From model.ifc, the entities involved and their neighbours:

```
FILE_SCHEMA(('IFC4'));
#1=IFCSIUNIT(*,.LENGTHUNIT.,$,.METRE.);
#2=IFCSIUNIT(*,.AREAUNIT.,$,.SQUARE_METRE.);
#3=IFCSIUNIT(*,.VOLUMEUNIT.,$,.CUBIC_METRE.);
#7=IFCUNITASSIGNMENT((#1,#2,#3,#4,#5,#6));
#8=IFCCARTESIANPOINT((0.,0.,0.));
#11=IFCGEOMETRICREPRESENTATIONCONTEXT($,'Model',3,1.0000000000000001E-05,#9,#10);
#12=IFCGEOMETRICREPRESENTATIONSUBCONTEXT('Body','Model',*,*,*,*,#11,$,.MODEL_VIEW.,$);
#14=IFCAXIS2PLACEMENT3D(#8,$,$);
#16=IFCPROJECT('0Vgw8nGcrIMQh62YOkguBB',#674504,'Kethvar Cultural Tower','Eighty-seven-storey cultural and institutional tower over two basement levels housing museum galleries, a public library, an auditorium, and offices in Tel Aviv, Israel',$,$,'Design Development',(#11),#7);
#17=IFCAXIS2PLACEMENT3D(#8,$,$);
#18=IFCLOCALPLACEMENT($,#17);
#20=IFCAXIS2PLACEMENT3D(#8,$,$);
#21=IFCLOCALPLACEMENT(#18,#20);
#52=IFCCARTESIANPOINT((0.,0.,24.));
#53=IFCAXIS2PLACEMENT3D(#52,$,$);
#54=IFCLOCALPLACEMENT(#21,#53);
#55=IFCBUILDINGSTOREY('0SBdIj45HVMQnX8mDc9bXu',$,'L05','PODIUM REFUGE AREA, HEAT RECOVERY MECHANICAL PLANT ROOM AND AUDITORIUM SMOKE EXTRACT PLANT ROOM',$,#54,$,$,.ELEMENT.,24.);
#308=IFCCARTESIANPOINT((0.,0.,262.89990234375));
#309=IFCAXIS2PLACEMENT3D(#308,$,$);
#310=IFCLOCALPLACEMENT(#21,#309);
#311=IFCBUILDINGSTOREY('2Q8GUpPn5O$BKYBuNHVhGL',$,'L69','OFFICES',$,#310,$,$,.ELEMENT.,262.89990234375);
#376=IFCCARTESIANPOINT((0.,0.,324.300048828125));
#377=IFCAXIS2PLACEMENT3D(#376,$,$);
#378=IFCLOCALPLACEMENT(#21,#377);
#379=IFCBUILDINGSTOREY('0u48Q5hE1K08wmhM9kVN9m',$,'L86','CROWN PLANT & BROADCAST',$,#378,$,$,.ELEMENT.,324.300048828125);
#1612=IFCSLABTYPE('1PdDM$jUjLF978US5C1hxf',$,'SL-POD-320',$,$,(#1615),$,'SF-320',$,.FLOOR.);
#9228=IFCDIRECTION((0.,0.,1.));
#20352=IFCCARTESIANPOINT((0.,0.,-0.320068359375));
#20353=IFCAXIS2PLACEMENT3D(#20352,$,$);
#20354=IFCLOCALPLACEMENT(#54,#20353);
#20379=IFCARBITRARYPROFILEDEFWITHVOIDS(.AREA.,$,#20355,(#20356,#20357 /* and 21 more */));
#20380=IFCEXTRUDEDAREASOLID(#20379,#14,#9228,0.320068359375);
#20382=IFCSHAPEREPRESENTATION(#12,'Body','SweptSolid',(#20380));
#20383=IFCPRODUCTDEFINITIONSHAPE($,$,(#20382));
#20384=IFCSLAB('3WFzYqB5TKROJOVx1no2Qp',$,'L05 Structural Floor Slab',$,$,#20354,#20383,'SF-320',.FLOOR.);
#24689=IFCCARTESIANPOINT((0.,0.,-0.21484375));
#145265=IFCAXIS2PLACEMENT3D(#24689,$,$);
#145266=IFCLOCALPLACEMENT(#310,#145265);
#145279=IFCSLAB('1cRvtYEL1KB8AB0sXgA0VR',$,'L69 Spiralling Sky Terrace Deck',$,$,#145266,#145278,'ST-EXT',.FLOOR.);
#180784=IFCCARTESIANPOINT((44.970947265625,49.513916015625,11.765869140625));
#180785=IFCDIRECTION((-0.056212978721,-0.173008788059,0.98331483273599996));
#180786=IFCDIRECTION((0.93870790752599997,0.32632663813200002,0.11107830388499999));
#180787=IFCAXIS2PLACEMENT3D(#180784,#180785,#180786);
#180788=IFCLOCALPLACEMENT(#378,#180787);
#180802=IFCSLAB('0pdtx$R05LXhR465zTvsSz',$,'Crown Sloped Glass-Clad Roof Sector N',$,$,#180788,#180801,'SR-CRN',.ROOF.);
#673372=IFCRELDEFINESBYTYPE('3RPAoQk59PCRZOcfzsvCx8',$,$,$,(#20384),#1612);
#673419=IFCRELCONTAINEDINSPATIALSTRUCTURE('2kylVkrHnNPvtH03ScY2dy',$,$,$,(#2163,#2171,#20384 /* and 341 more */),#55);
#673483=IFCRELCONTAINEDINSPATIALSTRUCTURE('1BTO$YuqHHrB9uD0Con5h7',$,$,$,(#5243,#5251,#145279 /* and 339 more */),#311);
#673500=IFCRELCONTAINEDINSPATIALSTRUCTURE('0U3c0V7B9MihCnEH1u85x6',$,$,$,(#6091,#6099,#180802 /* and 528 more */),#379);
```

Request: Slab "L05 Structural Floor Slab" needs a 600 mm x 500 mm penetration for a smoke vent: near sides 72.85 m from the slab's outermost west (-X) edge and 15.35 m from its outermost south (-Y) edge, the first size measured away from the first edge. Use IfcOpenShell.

```python
import numpy as np
import ifcopenshell
import ifcopenshell.api.feature
import ifcopenshell.api.geometry
import ifcopenshell.api.root
import ifcopenshell.geom
import ifcopenshell.util.placement
import ifcopenshell.util.representation
import ifcopenshell.util.shape
import ifcopenshell.util.unit

model = ifcopenshell.open("model.ifc")
unit_scale = ifcopenshell.util.unit.calculate_unit_scale(model)
settings = ifcopenshell.geom.settings()


def volume(element):
    """Net volume in cubic metres, openings subtracted."""
    shape = ifcopenshell.geom.create_shape(settings, element)
    return ifcopenshell.util.shape.get_volume(shape.geometry)


slab = model.by_id(20384)
before = volume(slab)

# Extent in the slab's own axes, in metres. The edges named are its -X and -Y sides.
slab_shape = ifcopenshell.geom.create_shape(settings, slab)
vertices = ifcopenshell.util.shape.get_vertices(slab_shape.geometry)
x_min, y_min, bottom = vertices.min(axis=0)
top = vertices[:, 2].max()

opening = ifcopenshell.api.root.create_entity(model, ifc_class="IfcOpeningElement", name="Smoke vent opening", predefined_type="OPENING")
context = ifcopenshell.util.representation.get_context(model, "Model", "Body", "MODEL_VIEW")
width, depth = 0.6, 0.5
outline = [(0.0, 0.0), (width, 0.0), (width, depth), (0.0, depth), (0.0, 0.0)]
# Overshoot both faces by 50 mm so the cut is clean.
shape = ifcopenshell.api.geometry.add_slab_representation(
    model, context=context, depth=top - bottom + 0.1, polyline=outline
)
ifcopenshell.api.geometry.assign_representation(model, product=opening, representation=shape)

matrix = ifcopenshell.util.placement.get_local_placement(slab.ObjectPlacement)
matrix[:, 3] = matrix @ np.append(np.array([x_min + 72.85, y_min + 15.35, bottom - 0.05]) / unit_scale, 1.0)
ifcopenshell.api.geometry.edit_object_placement(model, product=opening, matrix=matrix, is_si=False)
ifcopenshell.api.feature.add_feature(model, feature=opening, element=slab)

after = volume(slab)

print(f"slab volume {before:.3f} -> {after:.3f} m3")

model.write("model-out.ifc")
```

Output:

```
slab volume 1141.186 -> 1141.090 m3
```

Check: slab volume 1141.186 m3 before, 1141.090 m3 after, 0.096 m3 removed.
